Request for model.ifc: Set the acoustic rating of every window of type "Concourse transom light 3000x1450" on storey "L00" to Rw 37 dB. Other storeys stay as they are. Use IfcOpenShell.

First a look at what the model holds.

```python
import ifcopenshell
import ifcopenshell.util.element

model = ifcopenshell.open("model.ifc")
print(model.schema)
storey = next(s for s in model.by_type("IfcBuildingStorey") if s.Name == "L00")
windows = [e for e in ifcopenshell.util.element.get_decomposition(storey) if e.is_a("IfcWindow")]
seen = {}
for e in windows:
    element_type = ifcopenshell.util.element.get_type(e)
    key = (element_type.Name if element_type != e and element_type else None, ifcopenshell.util.element.get_pset(e, "Pset_WindowCommon", "AcousticRating"))
    seen[key] = seen.get(key, 0) + 1
for (name, value), count in sorted(seen.items(), key=str):
    print(count, "x", name, "|", value)
```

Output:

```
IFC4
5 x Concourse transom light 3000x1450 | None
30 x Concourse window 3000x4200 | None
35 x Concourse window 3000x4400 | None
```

```python
import ifcopenshell
import ifcopenshell.api.pset
import ifcopenshell.util.element

model = ifcopenshell.open("model.ifc")

storey = next(s for s in model.by_type("IfcBuildingStorey") if s.Name == "L00")
windows = [e for e in ifcopenshell.util.element.get_decomposition(storey) if e.is_a("IfcWindow")]

count = 0
for e in windows:
    element_type = ifcopenshell.util.element.get_type(e)
    if element_type in (None, e) or element_type.Name != "Concourse transom light 3000x1450":
        continue
    found = ifcopenshell.util.element.get_pset(e, "Pset_WindowCommon", should_inherit=False)
    if found:
        pset = model.by_id(found["id"])
        if len(ifcopenshell.util.element.get_elements_by_pset(pset)) > 1:
            pset = ifcopenshell.api.pset.unshare_pset(model, products=[e], pset=pset)[0]
    else:
        pset = ifcopenshell.api.pset.add_pset(model, product=e, name="Pset_WindowCommon")
    ifcopenshell.api.pset.edit_pset(model, pset=pset, properties={"AcousticRating": "Rw 37 dB"})
    count += 1

print(count, "windows updated")

model.write("model_updated.ifc")
```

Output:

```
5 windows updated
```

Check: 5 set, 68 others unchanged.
